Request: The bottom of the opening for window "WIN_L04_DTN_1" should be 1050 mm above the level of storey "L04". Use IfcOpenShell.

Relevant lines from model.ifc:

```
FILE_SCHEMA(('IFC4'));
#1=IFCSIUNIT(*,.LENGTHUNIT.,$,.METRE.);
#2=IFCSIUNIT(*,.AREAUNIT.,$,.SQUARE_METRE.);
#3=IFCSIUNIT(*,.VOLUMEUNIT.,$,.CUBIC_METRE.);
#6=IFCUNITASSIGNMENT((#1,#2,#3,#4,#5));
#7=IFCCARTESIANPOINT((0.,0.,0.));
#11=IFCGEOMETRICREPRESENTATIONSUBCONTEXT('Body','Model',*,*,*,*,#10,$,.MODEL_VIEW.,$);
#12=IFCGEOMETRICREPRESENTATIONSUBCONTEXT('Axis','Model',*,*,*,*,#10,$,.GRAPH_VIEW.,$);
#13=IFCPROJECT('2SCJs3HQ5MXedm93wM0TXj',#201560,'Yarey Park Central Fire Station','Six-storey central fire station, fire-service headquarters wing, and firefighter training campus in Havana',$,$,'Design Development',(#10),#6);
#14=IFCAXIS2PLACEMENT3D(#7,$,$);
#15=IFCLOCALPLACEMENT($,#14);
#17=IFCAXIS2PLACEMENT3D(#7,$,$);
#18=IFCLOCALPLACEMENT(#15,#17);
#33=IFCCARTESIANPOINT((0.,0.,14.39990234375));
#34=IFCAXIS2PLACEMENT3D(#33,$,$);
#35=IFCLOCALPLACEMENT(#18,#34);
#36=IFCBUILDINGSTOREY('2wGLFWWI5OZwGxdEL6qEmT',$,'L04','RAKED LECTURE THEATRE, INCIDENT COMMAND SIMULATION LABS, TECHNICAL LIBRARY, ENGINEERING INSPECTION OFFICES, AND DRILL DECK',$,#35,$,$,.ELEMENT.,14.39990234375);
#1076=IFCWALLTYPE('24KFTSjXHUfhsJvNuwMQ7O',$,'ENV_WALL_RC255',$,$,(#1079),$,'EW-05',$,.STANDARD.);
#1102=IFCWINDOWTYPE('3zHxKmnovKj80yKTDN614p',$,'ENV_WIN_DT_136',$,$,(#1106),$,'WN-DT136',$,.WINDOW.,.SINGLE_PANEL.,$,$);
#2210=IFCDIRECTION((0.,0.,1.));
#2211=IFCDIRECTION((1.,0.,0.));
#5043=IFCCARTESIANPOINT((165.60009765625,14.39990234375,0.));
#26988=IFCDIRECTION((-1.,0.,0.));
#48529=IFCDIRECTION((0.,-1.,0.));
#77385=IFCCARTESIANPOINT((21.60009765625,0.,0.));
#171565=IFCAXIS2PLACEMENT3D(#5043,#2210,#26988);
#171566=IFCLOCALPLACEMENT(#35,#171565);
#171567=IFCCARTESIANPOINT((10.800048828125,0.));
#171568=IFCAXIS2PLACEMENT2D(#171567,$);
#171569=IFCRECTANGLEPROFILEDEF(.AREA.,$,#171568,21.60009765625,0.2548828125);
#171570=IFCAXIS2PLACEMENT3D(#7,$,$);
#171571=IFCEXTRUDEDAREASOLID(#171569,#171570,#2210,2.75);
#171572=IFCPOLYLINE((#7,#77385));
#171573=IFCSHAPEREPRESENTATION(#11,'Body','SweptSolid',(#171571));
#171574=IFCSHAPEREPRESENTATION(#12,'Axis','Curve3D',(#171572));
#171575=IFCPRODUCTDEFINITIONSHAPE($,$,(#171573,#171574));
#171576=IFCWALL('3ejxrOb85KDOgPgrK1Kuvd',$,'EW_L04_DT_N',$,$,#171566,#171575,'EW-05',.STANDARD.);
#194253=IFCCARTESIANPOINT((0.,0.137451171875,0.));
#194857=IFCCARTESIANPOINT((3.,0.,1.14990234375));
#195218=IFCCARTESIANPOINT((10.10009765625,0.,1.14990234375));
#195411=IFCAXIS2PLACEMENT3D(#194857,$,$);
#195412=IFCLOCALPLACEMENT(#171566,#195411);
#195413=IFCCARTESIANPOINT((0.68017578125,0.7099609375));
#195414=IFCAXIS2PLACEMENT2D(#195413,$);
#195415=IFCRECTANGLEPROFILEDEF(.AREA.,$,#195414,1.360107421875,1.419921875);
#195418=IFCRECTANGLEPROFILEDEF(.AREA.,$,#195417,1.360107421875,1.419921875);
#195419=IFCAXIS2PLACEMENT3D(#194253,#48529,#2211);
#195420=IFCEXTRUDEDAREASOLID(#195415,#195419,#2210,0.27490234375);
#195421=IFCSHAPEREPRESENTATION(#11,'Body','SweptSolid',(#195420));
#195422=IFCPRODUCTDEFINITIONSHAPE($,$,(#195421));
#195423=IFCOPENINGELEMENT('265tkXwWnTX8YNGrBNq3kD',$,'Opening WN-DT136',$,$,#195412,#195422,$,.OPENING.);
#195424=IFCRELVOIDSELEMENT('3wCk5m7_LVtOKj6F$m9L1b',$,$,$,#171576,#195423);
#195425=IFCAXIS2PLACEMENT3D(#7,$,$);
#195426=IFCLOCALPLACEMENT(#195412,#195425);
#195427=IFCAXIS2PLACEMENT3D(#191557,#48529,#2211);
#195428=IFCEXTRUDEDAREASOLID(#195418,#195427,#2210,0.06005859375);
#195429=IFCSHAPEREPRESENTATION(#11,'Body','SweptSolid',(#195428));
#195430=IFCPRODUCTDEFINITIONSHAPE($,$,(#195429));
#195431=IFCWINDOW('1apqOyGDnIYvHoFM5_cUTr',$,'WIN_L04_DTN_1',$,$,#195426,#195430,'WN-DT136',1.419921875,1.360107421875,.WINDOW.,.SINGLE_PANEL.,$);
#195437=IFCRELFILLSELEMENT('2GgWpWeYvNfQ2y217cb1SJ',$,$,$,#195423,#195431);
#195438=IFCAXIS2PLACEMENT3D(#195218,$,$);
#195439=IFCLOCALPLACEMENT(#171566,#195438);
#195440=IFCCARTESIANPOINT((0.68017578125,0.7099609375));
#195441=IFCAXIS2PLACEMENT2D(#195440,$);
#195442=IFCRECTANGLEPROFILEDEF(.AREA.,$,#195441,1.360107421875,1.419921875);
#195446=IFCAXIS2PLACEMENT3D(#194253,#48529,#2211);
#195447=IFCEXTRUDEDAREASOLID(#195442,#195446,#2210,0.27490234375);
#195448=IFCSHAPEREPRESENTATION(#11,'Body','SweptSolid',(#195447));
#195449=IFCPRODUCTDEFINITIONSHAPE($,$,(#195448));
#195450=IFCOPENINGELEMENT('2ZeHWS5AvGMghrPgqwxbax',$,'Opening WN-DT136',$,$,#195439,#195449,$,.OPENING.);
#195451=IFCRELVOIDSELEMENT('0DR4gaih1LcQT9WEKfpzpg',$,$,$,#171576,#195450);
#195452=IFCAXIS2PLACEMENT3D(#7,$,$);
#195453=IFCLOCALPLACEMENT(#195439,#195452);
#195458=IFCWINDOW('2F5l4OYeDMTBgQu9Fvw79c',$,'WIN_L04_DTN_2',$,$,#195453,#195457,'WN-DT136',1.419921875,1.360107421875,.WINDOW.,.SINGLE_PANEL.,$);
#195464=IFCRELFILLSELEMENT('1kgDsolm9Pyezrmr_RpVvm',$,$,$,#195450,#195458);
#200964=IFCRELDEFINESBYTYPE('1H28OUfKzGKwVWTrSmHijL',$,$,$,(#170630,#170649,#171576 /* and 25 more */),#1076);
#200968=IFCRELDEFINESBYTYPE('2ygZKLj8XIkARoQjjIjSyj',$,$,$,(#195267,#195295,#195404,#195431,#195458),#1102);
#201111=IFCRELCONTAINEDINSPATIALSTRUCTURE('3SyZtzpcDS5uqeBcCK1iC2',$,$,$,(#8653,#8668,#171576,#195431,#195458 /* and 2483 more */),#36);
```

```python
import numpy as np
import ifcopenshell
import ifcopenshell.api.geometry
import ifcopenshell.geom
import ifcopenshell.util.element
import ifcopenshell.util.placement
import ifcopenshell.util.shape
import ifcopenshell.util.unit

model = ifcopenshell.open("model.ifc")
unit_scale = ifcopenshell.util.unit.calculate_unit_scale(model)

window = model.by_guid("1apqOyGDnIYvHoFM5_cUTr")
opening = window.FillsVoids[0].RelatingOpeningElement
storey = ifcopenshell.util.element.get_container(window, ifc_class="IfcBuildingStorey")
level = ifcopenshell.util.placement.get_local_placement(storey.ObjectPlacement)[2, 3]

# The opening's origin need not be at the sill, so measure its lowest point.
shape = ifcopenshell.geom.create_shape(ifcopenshell.geom.settings(), opening)
bottom = ifcopenshell.util.shape.get_shape_bottom_elevation(shape, shape.geometry) / unit_scale
dz = level + 1.05 - bottom

shift = np.array([0.0, 0.0, dz])
# The window is placed relative to its opening, so it follows when the opening moves.
matrix = ifcopenshell.util.placement.get_local_placement(opening.ObjectPlacement)
matrix[:3, 3] += shift
ifcopenshell.api.geometry.edit_object_placement(
    model, product=opening, matrix=matrix, is_si=False, should_transform_children=True
)

print(f"moved by {dz * unit_scale:+.3f} m")

model.write("model_rev.ifc")
```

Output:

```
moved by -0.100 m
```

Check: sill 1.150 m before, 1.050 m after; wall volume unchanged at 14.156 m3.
